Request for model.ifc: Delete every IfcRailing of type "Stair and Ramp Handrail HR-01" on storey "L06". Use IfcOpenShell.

First a look at what the model holds.

```python
import ifcopenshell
import ifcopenshell.util.element

model = ifcopenshell.open("model.ifc")
print(model.schema)
storey = next(s for s in model.by_type("IfcBuildingStorey") if s.Name == "L06")
railings = [e for e in ifcopenshell.util.element.get_decomposition(storey) if e.is_a("IfcRailing")]
seen = {}
for e in railings:
    element_type = ifcopenshell.util.element.get_type(e)
    name = element_type.Name if element_type not in (None, e) else None
    seen[name] = seen.get(name, 0) + 1
for name, count in sorted(seen.items(), key=str):
    print(count, "x", name)
```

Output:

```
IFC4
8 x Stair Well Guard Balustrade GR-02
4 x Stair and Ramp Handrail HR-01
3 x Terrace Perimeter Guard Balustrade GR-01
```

```python
import ifcopenshell
import ifcopenshell.api.root
import ifcopenshell.util.element

model = ifcopenshell.open("model.ifc")

storey = next(s for s in model.by_type("IfcBuildingStorey") if s.Name == "L06")
railings = [e for e in ifcopenshell.util.element.get_decomposition(storey) if e.is_a("IfcRailing")]
targets = [e for e in railings if (t := ifcopenshell.util.element.get_type(e)) not in (None, e) and t.Name == "Stair and Ramp Handrail HR-01"]

for e in targets:
    ifcopenshell.api.root.remove_product(model, product=e)
print(len(targets), "removed")

model.write("model-out.ifc")
```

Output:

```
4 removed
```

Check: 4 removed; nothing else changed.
